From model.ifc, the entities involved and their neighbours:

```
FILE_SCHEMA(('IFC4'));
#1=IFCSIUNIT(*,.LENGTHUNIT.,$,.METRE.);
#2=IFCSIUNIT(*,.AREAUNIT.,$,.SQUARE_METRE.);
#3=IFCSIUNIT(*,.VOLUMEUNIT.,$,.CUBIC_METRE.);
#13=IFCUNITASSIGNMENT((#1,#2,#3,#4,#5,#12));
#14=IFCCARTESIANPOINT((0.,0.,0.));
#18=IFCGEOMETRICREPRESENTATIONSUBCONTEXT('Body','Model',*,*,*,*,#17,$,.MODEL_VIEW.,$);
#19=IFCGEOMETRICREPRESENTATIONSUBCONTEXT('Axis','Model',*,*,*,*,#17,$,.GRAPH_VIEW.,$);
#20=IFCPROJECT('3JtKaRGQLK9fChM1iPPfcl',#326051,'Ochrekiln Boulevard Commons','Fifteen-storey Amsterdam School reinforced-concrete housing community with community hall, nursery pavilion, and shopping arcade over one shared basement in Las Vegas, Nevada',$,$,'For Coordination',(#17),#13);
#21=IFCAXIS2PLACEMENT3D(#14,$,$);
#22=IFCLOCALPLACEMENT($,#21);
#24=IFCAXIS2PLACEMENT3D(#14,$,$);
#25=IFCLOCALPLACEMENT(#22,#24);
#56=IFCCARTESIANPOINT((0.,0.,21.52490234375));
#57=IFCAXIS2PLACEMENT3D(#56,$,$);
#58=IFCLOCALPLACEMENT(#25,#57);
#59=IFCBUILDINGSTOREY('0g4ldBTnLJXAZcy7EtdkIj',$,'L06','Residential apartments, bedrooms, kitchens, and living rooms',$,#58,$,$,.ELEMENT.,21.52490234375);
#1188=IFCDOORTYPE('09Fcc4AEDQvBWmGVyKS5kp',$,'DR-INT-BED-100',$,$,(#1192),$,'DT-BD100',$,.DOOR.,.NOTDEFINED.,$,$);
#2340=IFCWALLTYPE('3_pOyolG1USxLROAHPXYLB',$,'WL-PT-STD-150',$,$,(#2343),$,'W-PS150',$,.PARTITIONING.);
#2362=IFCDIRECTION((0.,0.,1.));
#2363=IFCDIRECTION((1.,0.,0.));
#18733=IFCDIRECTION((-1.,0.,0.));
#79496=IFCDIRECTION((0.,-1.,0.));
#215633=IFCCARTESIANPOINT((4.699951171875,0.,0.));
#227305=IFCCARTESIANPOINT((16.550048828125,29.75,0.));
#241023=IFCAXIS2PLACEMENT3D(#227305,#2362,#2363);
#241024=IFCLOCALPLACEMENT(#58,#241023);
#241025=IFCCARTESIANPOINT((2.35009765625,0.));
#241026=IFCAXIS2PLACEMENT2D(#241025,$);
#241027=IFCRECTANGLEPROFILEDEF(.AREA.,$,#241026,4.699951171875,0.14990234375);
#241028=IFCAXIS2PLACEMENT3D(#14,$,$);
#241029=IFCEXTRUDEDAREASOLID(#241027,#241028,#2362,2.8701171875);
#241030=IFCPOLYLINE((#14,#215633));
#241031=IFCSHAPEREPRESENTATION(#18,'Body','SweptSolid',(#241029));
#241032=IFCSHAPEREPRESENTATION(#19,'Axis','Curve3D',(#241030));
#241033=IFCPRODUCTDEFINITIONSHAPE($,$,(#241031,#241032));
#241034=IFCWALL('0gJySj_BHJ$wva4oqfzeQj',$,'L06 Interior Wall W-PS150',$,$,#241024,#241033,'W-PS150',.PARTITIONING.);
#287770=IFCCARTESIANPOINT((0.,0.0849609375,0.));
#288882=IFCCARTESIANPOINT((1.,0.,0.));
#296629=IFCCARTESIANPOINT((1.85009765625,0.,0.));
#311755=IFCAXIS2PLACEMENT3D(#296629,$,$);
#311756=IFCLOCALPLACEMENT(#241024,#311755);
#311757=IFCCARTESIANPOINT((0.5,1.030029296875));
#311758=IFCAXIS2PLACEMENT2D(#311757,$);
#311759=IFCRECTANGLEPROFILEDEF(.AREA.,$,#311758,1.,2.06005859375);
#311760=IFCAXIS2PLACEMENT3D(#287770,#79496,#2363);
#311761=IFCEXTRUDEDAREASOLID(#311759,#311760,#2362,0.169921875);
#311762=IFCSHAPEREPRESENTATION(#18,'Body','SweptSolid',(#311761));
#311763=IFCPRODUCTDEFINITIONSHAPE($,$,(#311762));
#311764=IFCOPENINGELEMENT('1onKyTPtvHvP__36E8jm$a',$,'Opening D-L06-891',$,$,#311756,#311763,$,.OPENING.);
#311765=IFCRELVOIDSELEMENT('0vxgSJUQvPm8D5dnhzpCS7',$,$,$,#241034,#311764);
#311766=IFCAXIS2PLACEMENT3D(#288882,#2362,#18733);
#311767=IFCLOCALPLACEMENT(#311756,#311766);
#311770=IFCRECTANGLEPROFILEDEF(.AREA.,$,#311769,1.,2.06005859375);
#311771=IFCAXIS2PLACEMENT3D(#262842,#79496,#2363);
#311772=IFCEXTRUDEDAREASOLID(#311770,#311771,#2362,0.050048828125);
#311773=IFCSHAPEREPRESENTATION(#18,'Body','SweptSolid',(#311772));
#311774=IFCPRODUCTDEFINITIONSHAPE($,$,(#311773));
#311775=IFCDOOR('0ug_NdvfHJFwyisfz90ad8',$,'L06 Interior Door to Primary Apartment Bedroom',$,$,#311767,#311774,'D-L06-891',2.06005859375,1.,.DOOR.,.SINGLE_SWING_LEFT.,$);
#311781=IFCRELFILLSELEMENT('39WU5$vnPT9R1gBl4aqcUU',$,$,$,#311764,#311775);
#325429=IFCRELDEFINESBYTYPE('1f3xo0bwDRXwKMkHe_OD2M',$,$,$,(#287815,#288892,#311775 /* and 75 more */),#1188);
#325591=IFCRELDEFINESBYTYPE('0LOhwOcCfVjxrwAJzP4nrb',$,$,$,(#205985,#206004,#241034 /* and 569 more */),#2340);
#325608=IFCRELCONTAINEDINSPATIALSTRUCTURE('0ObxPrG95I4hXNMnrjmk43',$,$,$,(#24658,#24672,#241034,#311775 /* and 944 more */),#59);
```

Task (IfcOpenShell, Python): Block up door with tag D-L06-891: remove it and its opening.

```python
import ifcopenshell
import ifcopenshell.api.feature
import ifcopenshell.api.root
import ifcopenshell.geom
import ifcopenshell.util.shape

model = ifcopenshell.open("model.ifc")
settings = ifcopenshell.geom.settings()


def volume(element):
    """Net volume in cubic metres, openings subtracted."""
    shape = ifcopenshell.geom.create_shape(settings, element)
    return ifcopenshell.util.shape.get_volume(shape.geometry)


door = model.by_guid("0ug_NdvfHJFwyisfz90ad8")
opening = door.FillsVoids[0].RelatingOpeningElement
wall = opening.VoidsElements[0].RelatingBuildingElement
before = volume(wall)

ifcopenshell.api.root.remove_product(model, product=door)
ifcopenshell.api.feature.remove_feature(model, feature=opening)

after = volume(wall)

print(f"wall volume {before:.3f} -> {after:.3f} m3")

model.write("model-out.ifc")
```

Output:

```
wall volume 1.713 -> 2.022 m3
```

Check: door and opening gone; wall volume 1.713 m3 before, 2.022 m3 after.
